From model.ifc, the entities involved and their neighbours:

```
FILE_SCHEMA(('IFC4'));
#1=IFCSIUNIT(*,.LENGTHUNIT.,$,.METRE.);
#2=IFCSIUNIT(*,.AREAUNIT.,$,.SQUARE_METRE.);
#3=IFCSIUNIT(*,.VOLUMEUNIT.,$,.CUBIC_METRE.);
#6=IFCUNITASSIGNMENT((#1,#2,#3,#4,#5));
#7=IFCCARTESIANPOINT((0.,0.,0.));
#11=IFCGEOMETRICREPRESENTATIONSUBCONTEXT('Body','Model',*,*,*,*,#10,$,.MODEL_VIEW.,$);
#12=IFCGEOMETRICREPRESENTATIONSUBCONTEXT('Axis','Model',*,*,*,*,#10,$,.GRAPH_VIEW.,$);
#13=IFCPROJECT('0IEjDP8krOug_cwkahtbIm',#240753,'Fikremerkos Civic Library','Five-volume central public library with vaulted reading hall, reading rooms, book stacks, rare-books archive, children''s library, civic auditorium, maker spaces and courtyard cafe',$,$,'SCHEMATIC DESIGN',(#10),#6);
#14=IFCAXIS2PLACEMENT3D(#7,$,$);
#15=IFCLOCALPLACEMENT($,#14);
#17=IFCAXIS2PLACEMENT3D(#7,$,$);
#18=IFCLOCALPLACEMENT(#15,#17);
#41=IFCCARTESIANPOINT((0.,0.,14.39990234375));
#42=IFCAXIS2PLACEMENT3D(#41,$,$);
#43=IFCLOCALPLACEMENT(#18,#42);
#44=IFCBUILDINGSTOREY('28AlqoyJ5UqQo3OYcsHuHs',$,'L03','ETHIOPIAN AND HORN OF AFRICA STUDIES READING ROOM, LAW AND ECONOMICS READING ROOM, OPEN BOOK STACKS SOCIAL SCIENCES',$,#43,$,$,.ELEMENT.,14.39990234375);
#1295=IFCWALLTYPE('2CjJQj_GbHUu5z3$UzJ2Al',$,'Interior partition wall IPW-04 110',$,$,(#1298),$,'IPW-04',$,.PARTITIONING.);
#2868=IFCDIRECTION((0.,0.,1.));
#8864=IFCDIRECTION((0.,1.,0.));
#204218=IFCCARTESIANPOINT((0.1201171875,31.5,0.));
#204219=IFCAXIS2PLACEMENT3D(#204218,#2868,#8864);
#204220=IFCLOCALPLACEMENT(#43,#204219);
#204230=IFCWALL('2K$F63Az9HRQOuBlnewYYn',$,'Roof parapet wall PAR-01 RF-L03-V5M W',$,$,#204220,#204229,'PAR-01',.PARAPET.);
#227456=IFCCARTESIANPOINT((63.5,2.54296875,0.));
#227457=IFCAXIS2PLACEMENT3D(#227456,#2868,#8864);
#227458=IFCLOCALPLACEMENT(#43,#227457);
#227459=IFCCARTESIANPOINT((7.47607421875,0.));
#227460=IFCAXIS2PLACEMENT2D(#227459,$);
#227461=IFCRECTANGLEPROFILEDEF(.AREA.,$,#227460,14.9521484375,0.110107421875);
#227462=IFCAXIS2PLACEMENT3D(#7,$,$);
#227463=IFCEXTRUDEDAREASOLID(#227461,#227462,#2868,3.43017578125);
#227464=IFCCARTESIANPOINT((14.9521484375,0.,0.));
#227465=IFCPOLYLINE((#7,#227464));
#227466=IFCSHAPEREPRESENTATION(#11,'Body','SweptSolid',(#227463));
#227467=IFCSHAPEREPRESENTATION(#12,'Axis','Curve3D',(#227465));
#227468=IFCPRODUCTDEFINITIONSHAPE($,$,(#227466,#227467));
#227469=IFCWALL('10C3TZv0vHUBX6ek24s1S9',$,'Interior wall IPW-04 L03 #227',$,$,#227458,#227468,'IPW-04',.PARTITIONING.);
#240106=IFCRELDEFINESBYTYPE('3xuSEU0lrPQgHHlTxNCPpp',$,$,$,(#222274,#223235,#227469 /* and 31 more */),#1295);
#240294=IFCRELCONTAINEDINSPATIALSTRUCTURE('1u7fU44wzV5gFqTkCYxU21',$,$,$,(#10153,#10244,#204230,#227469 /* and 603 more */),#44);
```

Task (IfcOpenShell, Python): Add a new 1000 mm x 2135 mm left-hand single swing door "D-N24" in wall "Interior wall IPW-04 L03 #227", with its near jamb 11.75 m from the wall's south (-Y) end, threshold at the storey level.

```python
import numpy as np
import ifcopenshell
import ifcopenshell.api.feature
import ifcopenshell.api.geometry
import ifcopenshell.api.root
import ifcopenshell.api.spatial
import ifcopenshell.geom
import ifcopenshell.util.element
import ifcopenshell.util.placement
import ifcopenshell.util.representation
import ifcopenshell.util.shape
import ifcopenshell.util.unit

model = ifcopenshell.open("model.ifc")
unit_scale = ifcopenshell.util.unit.calculate_unit_scale(model)
settings = ifcopenshell.geom.settings()


def volume(element):
    """Net volume in cubic metres, openings subtracted."""
    shape = ifcopenshell.geom.create_shape(settings, element)
    return ifcopenshell.util.shape.get_volume(shape.geometry)


wall = model.by_guid("10C3TZv0vHUBX6ek24s1S9")
storey = ifcopenshell.util.element.get_container(wall, ifc_class="IfcBuildingStorey")
context = ifcopenshell.util.representation.get_context(model, "Model", "Body", "MODEL_VIEW")
before = volume(wall)

width, height, from_end, sill = 1, 2.135, 11.75, 0.0  # metres

# The wall runs along its own X axis, and the end named is its -X end.
wall_shape = ifcopenshell.geom.create_shape(settings, wall)
x, y, z = ifcopenshell.util.shape.get_vertices(wall_shape.geometry).T
start = x.min() + from_end
face, thickness = float(y.min()), float(y.max() - y.min())
wall_matrix = ifcopenshell.util.placement.get_local_placement(wall.ObjectPlacement)
level = ifcopenshell.util.placement.get_local_placement(storey.ObjectPlacement)[2, 3]


def in_wall(x, y):
    """Placement at x, y metres in the wall's axes, at sill height."""
    matrix = wall_matrix.copy()
    matrix[:, 3] = wall_matrix @ np.array([x / unit_scale, y / unit_scale, 0.0, 1.0])
    matrix[2, 3] = level + sill / unit_scale
    return matrix


# Opening: a box that overshoots both wall faces by 50 mm.
opening = ifcopenshell.api.root.create_entity(model, ifc_class="IfcOpeningElement", predefined_type="OPENING")
box = ifcopenshell.api.geometry.add_wall_representation(
    model, context=context, length=width, height=height, thickness=thickness + 0.1
)
ifcopenshell.api.geometry.assign_representation(model, product=opening, representation=box)
ifcopenshell.api.geometry.edit_object_placement(model, product=opening, matrix=in_wall(start, face - 0.05), is_si=False)
ifcopenshell.api.feature.add_feature(model, feature=opening, element=wall)

door = ifcopenshell.api.root.create_entity(model, ifc_class="IfcDoor", name="D-N24", predefined_type="DOOR")
door.OverallWidth, door.OverallHeight = width / unit_scale, height / unit_scale
door.OperationType = "SINGLE_SWING_LEFT"
body = ifcopenshell.api.geometry.add_door_representation(
    model,
    context=context,
    overall_width=door.OverallWidth,
    overall_height=door.OverallHeight,
    operation_type="SINGLE_SWING_LEFT",
    lining_properties={"LiningDepth": thickness / unit_scale, "ThresholdDepth": thickness / unit_scale},
)
ifcopenshell.api.geometry.assign_representation(model, product=door, representation=body)
ifcopenshell.api.spatial.assign_container(model, products=[door], relating_structure=storey)
ifcopenshell.api.feature.add_filling(model, opening=opening, element=door)

# The lining spans the wall, so the door starts at the wall face.
ifcopenshell.api.geometry.edit_object_placement(model, product=door, matrix=in_wall(start, face), is_si=False)

after = volume(wall)

print(f"wall volume {before:.3f} -> {after:.3f} m3")

model.write("model_edited.ifc")
```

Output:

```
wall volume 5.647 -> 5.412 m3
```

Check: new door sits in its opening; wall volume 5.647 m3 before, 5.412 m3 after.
